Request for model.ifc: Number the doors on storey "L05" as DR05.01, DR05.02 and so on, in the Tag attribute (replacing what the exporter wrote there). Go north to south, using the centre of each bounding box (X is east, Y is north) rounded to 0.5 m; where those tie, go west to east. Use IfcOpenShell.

First a look at what the model holds.

```python
import ifcopenshell
import ifcopenshell.util.element
import ifcopenshell.util.placement

model = ifcopenshell.open("model.ifc")
print(model.schema)
storey = next(s for s in model.by_type("IfcBuildingStorey") if s.Name == "L05")
doors = [e for e in ifcopenshell.util.element.get_decomposition(storey) if e.is_a("IfcDoor")]
for e in sorted(doors, key=lambda e: e.id()):
    origin = ifcopenshell.util.placement.get_local_placement(e.ObjectPlacement)[:3, 3]
    print(e.id(), e.Tag, e.Name, origin.round(2) + 0.0, sep=" | ")
```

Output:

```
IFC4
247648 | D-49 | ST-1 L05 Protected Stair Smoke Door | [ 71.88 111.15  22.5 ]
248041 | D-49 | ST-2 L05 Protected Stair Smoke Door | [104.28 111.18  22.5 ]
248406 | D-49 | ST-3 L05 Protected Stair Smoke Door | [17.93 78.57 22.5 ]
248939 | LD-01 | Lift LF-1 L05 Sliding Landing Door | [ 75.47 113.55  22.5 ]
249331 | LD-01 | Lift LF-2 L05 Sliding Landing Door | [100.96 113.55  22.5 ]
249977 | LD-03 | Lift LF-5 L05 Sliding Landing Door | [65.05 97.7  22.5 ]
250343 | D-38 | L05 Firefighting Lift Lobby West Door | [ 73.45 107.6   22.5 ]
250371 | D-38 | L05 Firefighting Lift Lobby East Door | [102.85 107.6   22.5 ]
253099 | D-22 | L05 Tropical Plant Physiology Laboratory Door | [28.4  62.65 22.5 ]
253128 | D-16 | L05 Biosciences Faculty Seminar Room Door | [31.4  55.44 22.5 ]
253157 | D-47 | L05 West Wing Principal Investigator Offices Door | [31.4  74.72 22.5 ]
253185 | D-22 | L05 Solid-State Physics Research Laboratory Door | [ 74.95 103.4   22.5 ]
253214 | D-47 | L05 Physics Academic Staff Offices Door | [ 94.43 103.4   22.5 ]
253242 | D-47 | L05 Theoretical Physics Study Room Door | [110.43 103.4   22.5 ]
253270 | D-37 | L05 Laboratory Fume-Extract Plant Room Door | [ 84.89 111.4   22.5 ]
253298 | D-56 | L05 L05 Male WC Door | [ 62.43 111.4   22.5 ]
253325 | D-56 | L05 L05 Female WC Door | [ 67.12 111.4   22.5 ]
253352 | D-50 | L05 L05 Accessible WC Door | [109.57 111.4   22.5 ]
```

```python
import ifcopenshell
import ifcopenshell.geom
import ifcopenshell.util.element
import ifcopenshell.util.shape

model = ifcopenshell.open("model.ifc")
settings = ifcopenshell.geom.settings()
settings.set("use-world-coords", True)


def centre(element):
    shape = ifcopenshell.geom.create_shape(settings, element)
    return ifcopenshell.util.shape.get_bbox_centroid(shape.geometry)


storey = next(s for s in model.by_type("IfcBuildingStorey") if s.Name == "L05")
doors = [e for e in ifcopenshell.util.element.get_decomposition(storey) if e.is_a("IfcDoor")]

# Insertion points can sit at a corner or the storey origin, so sort by the geometry (in metres).
centres = {e: centre(e) for e in doors}
doors.sort(key=lambda e: (-round(centres[e][1] / 0.5), centres[e][0]))

for i, e in enumerate(doors, start=1):
    number = f"DR05.{i:02d}"
    e.Tag = number
    print(e.id(), number)

model.write("model_edited.ifc")
```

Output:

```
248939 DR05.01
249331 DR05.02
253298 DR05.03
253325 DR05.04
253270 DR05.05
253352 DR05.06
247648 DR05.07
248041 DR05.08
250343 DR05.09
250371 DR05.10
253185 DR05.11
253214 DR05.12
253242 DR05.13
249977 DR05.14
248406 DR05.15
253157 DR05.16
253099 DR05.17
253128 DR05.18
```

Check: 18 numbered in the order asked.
